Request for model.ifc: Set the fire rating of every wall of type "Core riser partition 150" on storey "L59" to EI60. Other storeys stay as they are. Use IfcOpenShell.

First a look at what the model holds.

```python
import ifcopenshell
import ifcopenshell.util.element

model = ifcopenshell.open("model.ifc")
print(model.schema)
storey = next(s for s in model.by_type("IfcBuildingStorey") if s.Name == "L59")
walls = [e for e in ifcopenshell.util.element.get_decomposition(storey) if e.is_a("IfcWall")]
seen = {}
for e in walls:
    element_type = ifcopenshell.util.element.get_type(e)
    key = (element_type.Name if element_type != e and element_type else None, ifcopenshell.util.element.get_pset(e, "Pset_WallCommon", "FireRating"))
    seen[key] = seen.get(key, 0) + 1
for (name, value), count in sorted(seen.items(), key=str):
    print(count, "x", name, "|", value)
```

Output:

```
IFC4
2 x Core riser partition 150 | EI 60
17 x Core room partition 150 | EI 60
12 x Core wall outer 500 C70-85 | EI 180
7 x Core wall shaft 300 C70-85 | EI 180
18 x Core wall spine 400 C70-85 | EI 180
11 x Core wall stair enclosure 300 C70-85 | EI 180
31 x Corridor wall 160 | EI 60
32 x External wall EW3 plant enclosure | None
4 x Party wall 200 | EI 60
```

```python
import ifcopenshell
import ifcopenshell.api.pset
import ifcopenshell.util.element

model = ifcopenshell.open("model.ifc")

storey = next(s for s in model.by_type("IfcBuildingStorey") if s.Name == "L59")
walls = [e for e in ifcopenshell.util.element.get_decomposition(storey) if e.is_a("IfcWall")]

count = 0
for e in walls:
    element_type = ifcopenshell.util.element.get_type(e)
    if element_type in (None, e) or element_type.Name != "Core riser partition 150":
        continue
    found = ifcopenshell.util.element.get_pset(e, "Pset_WallCommon", should_inherit=False)
    if found:
        pset = model.by_id(found["id"])
        if len(ifcopenshell.util.element.get_elements_by_pset(pset)) > 1:
            pset = ifcopenshell.api.pset.unshare_pset(model, products=[e], pset=pset)[0]
    else:
        pset = ifcopenshell.api.pset.add_pset(model, product=e, name="Pset_WallCommon")
    ifcopenshell.api.pset.edit_pset(model, pset=pset, properties={"FireRating": "EI60"})
    count += 1

print(count, "walls updated")

model.write("model-out.ifc")
```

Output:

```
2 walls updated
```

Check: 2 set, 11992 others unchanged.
